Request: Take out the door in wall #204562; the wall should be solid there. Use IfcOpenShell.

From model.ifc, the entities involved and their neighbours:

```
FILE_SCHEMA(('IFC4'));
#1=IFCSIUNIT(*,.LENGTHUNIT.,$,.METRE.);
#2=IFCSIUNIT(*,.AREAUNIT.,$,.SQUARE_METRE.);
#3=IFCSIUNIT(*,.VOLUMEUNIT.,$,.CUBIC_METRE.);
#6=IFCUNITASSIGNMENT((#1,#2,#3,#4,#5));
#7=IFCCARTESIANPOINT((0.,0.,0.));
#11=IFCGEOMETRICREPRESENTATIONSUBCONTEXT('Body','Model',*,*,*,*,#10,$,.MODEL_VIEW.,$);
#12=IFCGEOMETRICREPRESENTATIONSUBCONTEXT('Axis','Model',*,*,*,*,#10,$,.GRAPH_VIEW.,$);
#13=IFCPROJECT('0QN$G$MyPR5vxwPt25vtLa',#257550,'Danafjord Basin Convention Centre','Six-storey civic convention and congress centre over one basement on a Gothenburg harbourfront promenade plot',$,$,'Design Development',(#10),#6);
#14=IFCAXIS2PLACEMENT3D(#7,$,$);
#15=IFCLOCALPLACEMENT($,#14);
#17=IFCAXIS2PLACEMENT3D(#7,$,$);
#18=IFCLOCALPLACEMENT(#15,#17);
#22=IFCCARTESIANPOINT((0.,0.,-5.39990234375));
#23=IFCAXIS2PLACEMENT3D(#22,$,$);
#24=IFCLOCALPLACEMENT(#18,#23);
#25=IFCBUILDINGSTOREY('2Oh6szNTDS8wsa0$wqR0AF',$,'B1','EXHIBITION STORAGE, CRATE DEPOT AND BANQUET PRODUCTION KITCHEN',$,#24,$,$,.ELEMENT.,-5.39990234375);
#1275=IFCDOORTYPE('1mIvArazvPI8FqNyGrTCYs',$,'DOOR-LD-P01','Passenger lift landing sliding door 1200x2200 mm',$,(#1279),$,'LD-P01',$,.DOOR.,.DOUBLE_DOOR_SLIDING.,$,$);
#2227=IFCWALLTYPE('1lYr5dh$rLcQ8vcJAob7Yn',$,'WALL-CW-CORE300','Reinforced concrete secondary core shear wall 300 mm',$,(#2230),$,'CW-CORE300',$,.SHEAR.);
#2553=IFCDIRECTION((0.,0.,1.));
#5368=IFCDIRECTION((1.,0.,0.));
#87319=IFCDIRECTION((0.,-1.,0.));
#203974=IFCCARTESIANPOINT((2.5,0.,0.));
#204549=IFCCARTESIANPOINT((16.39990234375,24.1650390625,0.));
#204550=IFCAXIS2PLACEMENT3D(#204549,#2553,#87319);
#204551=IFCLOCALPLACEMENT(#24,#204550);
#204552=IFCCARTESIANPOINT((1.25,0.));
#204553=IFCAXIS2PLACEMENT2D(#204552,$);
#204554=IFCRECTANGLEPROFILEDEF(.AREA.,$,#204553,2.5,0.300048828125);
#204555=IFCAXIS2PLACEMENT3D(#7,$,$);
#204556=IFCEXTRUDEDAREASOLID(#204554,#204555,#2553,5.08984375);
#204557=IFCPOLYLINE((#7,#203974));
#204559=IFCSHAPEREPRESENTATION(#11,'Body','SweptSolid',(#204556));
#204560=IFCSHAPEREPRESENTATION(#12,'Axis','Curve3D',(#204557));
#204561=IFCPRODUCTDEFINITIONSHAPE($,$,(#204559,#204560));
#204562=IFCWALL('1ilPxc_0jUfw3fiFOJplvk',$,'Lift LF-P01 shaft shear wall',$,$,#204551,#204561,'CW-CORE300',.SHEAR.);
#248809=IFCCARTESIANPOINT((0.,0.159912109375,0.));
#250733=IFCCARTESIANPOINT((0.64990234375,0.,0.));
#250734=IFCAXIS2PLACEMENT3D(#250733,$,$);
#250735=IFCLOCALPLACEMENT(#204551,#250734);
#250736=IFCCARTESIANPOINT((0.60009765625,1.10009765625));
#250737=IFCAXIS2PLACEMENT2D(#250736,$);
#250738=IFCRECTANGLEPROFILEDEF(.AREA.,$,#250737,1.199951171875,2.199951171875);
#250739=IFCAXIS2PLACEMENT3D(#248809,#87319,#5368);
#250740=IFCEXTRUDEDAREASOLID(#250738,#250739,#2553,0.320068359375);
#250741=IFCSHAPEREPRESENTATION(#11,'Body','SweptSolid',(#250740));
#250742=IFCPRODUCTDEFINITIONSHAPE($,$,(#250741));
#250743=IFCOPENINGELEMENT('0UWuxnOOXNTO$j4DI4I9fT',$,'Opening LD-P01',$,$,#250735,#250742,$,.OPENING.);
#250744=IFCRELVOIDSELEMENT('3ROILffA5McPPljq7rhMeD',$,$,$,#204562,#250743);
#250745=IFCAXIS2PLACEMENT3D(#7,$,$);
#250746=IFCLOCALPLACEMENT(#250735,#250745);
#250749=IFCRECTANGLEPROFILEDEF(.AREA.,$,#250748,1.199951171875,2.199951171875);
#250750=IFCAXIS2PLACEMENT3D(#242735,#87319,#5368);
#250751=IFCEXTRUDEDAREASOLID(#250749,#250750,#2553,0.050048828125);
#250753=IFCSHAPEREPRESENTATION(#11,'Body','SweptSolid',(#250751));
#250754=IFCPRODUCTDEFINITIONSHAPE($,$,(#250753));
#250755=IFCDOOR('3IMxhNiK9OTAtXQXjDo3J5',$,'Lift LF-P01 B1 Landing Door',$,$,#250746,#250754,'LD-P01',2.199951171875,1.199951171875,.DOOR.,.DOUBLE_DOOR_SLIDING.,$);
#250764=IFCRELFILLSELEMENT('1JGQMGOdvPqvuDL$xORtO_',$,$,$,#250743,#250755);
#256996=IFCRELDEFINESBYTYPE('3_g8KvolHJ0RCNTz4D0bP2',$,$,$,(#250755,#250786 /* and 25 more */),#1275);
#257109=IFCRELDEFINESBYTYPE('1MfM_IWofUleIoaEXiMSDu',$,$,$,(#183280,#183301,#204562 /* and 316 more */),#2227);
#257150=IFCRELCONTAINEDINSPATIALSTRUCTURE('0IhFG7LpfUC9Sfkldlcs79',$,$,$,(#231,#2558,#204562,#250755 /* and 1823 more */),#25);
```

```python
import ifcopenshell
import ifcopenshell.api.feature
import ifcopenshell.api.root
import ifcopenshell.geom
import ifcopenshell.util.shape

model = ifcopenshell.open("model.ifc")
settings = ifcopenshell.geom.settings()


def volume(element):
    """Net volume in cubic metres, openings subtracted."""
    shape = ifcopenshell.geom.create_shape(settings, element)
    return ifcopenshell.util.shape.get_volume(shape.geometry)


door = model.by_id(250755)
opening = door.FillsVoids[0].RelatingOpeningElement
wall = opening.VoidsElements[0].RelatingBuildingElement
before = volume(wall)

ifcopenshell.api.root.remove_product(model, product=door)
ifcopenshell.api.feature.remove_feature(model, feature=opening)

after = volume(wall)

print(f"wall volume {before:.3f} -> {after:.3f} m3")

model.write("model_updated.ifc")
```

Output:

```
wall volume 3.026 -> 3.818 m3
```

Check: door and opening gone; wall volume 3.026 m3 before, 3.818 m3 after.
